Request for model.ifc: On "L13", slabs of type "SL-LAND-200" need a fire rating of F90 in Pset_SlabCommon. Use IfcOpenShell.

First a look at what the model holds.

```python
import ifcopenshell
import ifcopenshell.util.element

model = ifcopenshell.open("model.ifc")
print(model.schema)
storey = next(s for s in model.by_type("IfcBuildingStorey") if s.Name == "L13")
slabs = [e for e in ifcopenshell.util.element.get_decomposition(storey) if e.is_a("IfcSlab")]
seen = {}
for e in slabs:
    element_type = ifcopenshell.util.element.get_type(e)
    key = (element_type.Name if element_type != e and element_type else None, ifcopenshell.util.element.get_pset(e, "Pset_SlabCommon", "FireRating"))
    seen[key] = seen.get(key, 0) + 1
for (name, value), count in sorted(seen.items(), key=str):
    print(count, "x", name, "|", value)
```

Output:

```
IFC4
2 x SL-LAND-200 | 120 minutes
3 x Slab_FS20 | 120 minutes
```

```python
import ifcopenshell
import ifcopenshell.api.pset
import ifcopenshell.util.element

model = ifcopenshell.open("model.ifc")

storey = next(s for s in model.by_type("IfcBuildingStorey") if s.Name == "L13")
slabs = [e for e in ifcopenshell.util.element.get_decomposition(storey) if e.is_a("IfcSlab")]

count = 0
for e in slabs:
    element_type = ifcopenshell.util.element.get_type(e)
    if element_type in (None, e) or element_type.Name != "SL-LAND-200":
        continue
    # add_pset returns the element's existing set when there is one.
    pset = ifcopenshell.api.pset.add_pset(model, product=e, name="Pset_SlabCommon")
    ifcopenshell.api.pset.edit_pset(model, pset=pset, properties={"FireRating": "F90"})
    count += 1

print(count, "slabs updated")

model.write("model-out.ifc")
```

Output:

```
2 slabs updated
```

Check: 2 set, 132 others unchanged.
